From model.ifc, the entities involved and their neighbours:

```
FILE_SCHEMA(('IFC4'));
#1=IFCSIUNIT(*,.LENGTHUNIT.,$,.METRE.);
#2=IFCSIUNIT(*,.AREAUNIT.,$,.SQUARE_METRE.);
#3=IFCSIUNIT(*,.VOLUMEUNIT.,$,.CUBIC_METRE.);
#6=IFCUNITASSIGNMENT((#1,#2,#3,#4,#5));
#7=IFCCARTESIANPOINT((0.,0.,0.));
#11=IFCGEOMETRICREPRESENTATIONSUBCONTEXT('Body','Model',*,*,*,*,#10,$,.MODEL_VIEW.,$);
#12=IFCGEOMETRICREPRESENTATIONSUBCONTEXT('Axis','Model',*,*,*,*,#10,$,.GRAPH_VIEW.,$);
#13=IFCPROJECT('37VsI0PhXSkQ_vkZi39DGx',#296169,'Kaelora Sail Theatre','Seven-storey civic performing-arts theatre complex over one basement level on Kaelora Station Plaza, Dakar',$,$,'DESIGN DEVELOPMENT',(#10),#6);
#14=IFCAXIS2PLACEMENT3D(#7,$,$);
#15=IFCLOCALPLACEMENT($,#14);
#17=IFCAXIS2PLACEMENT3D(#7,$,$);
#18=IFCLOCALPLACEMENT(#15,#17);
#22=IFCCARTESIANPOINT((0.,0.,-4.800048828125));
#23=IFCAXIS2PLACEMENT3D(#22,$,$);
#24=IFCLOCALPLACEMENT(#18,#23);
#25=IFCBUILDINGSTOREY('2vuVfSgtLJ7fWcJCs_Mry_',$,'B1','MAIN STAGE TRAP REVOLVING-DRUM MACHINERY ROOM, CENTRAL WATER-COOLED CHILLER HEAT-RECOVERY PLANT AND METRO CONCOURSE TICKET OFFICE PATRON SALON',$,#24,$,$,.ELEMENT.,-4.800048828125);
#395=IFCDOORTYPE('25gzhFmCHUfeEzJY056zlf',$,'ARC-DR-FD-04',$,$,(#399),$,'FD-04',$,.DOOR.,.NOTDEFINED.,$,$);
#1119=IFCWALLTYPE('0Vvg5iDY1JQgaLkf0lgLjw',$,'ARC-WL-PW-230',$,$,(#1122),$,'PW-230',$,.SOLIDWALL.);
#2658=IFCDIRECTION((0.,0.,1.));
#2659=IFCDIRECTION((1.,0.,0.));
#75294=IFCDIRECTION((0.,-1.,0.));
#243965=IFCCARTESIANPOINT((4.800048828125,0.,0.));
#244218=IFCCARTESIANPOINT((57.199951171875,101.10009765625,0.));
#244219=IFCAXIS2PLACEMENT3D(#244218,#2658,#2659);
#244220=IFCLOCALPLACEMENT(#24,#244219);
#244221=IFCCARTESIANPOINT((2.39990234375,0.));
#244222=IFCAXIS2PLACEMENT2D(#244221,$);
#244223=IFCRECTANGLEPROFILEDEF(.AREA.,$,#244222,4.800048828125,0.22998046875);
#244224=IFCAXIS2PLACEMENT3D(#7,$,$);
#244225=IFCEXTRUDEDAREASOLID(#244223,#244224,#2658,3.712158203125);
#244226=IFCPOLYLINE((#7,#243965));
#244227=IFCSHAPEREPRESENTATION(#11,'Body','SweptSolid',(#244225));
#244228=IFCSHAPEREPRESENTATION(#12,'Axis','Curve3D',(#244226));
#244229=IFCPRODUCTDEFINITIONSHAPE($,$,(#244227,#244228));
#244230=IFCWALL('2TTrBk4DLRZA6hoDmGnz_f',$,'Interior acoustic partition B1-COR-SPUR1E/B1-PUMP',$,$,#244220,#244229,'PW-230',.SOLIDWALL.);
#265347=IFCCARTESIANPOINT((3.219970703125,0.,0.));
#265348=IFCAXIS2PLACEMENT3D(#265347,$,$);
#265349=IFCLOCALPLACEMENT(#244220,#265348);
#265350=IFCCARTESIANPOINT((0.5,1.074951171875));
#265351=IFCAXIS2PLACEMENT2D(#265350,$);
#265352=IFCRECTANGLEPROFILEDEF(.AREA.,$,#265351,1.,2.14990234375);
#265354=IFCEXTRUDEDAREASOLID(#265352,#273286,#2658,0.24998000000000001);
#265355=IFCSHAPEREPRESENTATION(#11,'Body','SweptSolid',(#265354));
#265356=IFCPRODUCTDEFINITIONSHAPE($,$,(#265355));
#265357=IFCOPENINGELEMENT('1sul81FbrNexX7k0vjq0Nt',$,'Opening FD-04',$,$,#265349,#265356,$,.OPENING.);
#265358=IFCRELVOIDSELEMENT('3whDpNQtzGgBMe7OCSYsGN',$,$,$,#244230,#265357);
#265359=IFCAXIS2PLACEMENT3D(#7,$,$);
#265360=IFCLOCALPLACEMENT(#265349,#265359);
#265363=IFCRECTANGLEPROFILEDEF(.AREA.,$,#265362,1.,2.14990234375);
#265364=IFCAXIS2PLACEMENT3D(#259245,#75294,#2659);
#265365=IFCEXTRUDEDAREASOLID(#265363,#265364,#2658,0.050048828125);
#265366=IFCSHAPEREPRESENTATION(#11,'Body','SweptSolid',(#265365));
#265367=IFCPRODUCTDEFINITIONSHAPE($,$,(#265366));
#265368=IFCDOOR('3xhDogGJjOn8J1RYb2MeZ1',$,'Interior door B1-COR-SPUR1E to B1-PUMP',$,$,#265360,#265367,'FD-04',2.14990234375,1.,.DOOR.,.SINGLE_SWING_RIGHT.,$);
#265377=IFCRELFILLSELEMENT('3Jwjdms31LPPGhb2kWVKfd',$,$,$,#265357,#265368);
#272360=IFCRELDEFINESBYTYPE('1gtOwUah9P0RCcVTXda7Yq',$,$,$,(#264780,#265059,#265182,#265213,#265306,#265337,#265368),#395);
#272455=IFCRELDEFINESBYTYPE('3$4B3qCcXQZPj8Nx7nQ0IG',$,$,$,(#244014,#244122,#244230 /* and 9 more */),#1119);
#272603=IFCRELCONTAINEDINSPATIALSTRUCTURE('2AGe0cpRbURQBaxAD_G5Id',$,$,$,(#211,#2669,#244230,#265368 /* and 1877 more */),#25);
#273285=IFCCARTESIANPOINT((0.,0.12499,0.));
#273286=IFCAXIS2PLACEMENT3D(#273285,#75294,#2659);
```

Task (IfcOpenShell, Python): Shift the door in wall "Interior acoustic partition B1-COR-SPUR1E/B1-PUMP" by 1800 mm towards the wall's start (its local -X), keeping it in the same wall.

```python
import ifcopenshell
import ifcopenshell.api.geometry
import ifcopenshell.util.placement
import ifcopenshell.util.unit

model = ifcopenshell.open("model.ifc")
unit_scale = ifcopenshell.util.unit.calculate_unit_scale(model)

door = model.by_guid("3xhDogGJjOn8J1RYb2MeZ1")
opening = door.FillsVoids[0].RelatingOpeningElement
wall = opening.VoidsElements[0].RelatingBuildingElement

wall_matrix = ifcopenshell.util.placement.get_local_placement(wall.ObjectPlacement)
shift = wall_matrix[:3, 0] * -1.8 / unit_scale
before = ifcopenshell.util.placement.get_local_placement(door.ObjectPlacement)[:3, 3].copy()

# The door is placed relative to its opening, so it follows when the opening moves.
matrix = ifcopenshell.util.placement.get_local_placement(opening.ObjectPlacement)
matrix[:3, 3] += shift
ifcopenshell.api.geometry.edit_object_placement(
    model, product=opening, matrix=matrix, is_si=False, should_transform_children=True
)

after = ifcopenshell.util.placement.get_local_placement(door.ObjectPlacement)[:3, 3]
print("door moved by", (after - before).round(3) + 0.0)

model.write("model_updated.ifc")
```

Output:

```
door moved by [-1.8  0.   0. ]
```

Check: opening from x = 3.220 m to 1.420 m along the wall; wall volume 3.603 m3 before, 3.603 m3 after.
